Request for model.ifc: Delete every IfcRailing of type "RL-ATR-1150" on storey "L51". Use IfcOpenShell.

First a look at what the model holds.

```python
import ifcopenshell
import ifcopenshell.util.element

model = ifcopenshell.open("model.ifc")
print(model.schema)
storey = next(s for s in model.by_type("IfcBuildingStorey") if s.Name == "L51")
railings = [e for e in ifcopenshell.util.element.get_decomposition(storey) if e.is_a("IfcRailing")]
seen = {}
for e in railings:
    element_type = ifcopenshell.util.element.get_type(e)
    name = element_type.Name if element_type not in (None, e) else None
    seen[name] = seen.get(name, 0) + 1
for name, count in sorted(seen.items(), key=str):
    print(count, "x", name)
```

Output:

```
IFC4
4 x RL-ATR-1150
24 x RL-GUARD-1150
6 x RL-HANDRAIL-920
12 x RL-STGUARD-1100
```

```python
import ifcopenshell
import ifcopenshell.api.root
import ifcopenshell.util.element

model = ifcopenshell.open("model.ifc")

storey = next(s for s in model.by_type("IfcBuildingStorey") if s.Name == "L51")
railings = [e for e in ifcopenshell.util.element.get_decomposition(storey) if e.is_a("IfcRailing")]
targets = [e for e in railings if (t := ifcopenshell.util.element.get_type(e)) not in (None, e) and t.Name == "RL-ATR-1150"]

for e in targets:
    ifcopenshell.api.root.remove_product(model, product=e)
print(len(targets), "removed")

model.write("model_v2.ifc")
```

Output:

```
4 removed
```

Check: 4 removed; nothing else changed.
